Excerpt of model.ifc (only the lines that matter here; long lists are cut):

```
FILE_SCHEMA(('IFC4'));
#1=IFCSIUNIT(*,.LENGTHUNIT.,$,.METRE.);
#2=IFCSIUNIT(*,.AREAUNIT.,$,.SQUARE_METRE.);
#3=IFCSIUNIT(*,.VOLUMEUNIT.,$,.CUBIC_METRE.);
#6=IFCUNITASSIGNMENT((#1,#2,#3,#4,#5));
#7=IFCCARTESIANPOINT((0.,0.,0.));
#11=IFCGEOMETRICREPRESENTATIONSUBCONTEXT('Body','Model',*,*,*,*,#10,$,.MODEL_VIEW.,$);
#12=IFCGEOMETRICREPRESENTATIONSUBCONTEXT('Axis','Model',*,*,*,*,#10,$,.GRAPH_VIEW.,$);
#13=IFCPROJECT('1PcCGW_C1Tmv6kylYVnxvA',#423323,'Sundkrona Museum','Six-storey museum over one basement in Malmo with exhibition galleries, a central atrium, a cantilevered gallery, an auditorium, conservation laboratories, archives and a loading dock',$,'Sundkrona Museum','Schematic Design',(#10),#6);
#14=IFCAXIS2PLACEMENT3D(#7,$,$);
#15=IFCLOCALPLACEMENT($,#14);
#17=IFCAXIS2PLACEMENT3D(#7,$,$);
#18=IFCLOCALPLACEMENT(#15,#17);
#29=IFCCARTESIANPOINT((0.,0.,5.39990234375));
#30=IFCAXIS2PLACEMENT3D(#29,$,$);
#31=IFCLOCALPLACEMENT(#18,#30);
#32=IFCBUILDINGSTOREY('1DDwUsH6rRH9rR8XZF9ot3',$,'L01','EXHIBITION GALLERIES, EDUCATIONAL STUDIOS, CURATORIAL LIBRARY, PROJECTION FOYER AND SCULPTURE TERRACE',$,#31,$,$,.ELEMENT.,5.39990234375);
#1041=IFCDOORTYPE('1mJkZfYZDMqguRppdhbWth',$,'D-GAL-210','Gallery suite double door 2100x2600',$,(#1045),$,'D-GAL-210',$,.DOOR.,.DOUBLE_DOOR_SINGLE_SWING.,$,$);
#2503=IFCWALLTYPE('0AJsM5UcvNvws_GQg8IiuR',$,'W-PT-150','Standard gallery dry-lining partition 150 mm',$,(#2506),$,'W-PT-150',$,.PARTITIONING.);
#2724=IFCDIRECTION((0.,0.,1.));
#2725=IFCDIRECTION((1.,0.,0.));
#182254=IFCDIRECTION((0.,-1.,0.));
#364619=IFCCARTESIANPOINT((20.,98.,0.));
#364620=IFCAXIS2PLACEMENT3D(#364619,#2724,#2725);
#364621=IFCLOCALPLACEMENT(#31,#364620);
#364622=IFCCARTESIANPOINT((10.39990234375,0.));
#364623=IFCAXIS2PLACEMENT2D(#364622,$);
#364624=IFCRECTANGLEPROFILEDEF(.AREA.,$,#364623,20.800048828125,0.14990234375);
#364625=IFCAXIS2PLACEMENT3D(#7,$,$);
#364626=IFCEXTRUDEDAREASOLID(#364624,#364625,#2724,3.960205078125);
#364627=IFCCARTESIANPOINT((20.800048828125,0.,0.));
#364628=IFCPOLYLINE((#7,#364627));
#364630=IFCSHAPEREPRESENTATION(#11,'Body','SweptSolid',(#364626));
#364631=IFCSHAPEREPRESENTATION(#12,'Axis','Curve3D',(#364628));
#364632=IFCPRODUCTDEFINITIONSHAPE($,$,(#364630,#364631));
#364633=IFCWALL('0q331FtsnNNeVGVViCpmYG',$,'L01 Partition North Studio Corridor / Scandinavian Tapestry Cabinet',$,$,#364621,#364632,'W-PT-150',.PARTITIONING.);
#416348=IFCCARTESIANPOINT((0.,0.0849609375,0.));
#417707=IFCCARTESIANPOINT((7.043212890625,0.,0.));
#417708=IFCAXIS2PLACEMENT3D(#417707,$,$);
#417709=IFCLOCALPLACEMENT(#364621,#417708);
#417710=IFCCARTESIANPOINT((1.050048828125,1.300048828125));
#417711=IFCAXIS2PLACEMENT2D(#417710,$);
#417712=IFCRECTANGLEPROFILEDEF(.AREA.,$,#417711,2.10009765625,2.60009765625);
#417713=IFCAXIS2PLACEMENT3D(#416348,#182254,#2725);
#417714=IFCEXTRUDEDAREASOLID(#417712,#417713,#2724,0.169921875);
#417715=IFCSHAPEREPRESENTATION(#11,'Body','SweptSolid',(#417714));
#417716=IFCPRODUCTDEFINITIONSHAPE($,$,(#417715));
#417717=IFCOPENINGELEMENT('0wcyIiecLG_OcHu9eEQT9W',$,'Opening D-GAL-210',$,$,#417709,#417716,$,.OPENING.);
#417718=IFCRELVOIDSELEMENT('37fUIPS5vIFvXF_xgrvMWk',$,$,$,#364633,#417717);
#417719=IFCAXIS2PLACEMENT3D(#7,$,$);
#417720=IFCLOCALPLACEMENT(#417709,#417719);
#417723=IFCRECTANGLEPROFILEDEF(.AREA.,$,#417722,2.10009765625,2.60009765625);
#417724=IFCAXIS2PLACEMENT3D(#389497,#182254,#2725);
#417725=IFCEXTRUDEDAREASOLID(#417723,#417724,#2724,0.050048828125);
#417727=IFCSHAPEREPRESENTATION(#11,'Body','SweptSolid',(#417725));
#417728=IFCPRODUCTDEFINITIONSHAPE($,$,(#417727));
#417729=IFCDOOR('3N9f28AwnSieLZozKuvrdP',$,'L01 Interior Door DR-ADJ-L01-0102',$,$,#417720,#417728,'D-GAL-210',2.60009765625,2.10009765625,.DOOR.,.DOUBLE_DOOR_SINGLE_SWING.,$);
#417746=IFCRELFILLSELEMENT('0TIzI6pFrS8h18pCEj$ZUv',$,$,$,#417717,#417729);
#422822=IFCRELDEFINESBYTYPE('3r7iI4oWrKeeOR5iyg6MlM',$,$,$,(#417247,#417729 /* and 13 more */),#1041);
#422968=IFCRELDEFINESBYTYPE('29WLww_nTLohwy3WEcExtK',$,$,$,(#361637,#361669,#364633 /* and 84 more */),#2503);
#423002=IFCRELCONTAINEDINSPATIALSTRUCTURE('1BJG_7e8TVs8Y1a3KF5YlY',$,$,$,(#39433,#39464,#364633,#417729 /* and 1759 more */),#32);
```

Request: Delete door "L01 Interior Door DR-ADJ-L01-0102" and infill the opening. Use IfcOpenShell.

```python
import ifcopenshell
import ifcopenshell.api.feature
import ifcopenshell.api.root
import ifcopenshell.geom
import ifcopenshell.util.shape

model = ifcopenshell.open("model.ifc")
settings = ifcopenshell.geom.settings()


def volume(element):
    """Net volume in cubic metres, openings subtracted."""
    shape = ifcopenshell.geom.create_shape(settings, element)
    return ifcopenshell.util.shape.get_volume(shape.geometry)


door = model.by_guid("3N9f28AwnSieLZozKuvrdP")
opening = door.FillsVoids[0].RelatingOpeningElement
wall = opening.VoidsElements[0].RelatingBuildingElement
before = volume(wall)

ifcopenshell.api.root.remove_product(model, product=door)
ifcopenshell.api.feature.remove_feature(model, feature=opening)

after = volume(wall)

print(f"wall volume {before:.3f} -> {after:.3f} m3")

model.write("model_edited.ifc")
```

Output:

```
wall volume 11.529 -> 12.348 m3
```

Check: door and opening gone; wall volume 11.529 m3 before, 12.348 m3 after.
